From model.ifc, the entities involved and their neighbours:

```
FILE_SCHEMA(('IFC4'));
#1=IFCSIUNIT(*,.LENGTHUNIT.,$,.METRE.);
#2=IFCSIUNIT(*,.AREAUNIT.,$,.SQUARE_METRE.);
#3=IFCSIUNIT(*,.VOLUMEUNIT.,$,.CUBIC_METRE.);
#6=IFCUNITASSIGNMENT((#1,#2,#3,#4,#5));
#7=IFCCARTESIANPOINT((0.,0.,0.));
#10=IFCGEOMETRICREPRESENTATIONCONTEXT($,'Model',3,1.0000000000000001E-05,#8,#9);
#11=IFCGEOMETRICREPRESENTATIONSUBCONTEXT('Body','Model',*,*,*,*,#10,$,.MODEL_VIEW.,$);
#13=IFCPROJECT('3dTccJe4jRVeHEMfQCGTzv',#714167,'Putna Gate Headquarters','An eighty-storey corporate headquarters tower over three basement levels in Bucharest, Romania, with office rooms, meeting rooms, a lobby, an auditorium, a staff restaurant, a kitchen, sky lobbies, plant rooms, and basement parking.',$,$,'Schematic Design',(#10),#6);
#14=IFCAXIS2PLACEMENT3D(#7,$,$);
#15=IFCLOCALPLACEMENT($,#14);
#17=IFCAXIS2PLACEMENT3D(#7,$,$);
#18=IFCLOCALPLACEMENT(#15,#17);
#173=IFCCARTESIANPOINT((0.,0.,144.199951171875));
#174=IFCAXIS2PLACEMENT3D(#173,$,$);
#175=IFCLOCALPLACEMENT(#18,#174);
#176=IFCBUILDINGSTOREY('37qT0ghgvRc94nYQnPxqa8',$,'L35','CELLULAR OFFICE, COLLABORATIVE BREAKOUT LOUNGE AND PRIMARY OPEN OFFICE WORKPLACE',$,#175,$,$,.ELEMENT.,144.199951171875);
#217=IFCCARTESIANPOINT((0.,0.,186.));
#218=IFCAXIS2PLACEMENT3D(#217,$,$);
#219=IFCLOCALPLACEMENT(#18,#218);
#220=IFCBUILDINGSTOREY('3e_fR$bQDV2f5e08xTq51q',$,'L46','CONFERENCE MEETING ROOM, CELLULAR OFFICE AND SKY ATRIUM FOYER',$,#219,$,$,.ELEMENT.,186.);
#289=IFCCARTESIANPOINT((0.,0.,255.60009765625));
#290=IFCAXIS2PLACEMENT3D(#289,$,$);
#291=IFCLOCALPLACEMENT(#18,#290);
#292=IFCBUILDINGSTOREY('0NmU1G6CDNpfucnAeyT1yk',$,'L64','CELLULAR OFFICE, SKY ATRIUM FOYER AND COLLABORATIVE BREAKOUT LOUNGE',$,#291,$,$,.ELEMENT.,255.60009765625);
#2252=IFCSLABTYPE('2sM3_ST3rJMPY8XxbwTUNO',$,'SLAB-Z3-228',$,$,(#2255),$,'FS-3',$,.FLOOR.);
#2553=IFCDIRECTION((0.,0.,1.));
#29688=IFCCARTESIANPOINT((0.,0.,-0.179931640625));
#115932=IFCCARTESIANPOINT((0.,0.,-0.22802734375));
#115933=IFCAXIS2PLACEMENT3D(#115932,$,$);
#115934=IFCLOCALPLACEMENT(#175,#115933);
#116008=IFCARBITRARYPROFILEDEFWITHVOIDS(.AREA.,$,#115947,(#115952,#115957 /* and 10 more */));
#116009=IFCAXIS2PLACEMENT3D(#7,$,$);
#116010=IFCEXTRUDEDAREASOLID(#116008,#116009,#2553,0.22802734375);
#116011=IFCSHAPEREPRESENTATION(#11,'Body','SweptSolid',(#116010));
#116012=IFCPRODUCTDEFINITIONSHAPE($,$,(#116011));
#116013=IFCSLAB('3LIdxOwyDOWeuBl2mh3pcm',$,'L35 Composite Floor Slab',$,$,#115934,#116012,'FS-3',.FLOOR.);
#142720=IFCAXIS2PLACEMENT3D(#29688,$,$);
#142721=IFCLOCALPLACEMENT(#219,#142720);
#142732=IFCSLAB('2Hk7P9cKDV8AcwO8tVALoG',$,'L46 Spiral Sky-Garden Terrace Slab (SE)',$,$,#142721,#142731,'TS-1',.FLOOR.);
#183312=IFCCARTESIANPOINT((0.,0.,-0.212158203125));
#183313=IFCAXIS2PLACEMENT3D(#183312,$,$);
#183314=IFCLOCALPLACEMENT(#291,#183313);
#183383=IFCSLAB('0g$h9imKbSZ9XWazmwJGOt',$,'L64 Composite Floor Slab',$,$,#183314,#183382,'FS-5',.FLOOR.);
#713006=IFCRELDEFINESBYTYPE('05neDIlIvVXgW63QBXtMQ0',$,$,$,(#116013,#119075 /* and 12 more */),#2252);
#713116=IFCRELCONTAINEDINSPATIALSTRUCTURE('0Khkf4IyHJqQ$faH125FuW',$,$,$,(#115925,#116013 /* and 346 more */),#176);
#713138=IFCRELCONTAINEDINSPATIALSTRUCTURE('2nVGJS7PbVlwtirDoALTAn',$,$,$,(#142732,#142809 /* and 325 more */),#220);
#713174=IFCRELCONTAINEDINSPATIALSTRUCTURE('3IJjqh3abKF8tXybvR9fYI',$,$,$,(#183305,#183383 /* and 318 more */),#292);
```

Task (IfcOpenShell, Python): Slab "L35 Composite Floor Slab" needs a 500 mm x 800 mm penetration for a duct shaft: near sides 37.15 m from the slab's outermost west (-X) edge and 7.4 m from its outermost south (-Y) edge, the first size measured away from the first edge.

```python
import numpy as np
import ifcopenshell
import ifcopenshell.api.feature
import ifcopenshell.api.geometry
import ifcopenshell.api.root
import ifcopenshell.geom
import ifcopenshell.util.placement
import ifcopenshell.util.representation
import ifcopenshell.util.shape
import ifcopenshell.util.unit

model = ifcopenshell.open("model.ifc")
unit_scale = ifcopenshell.util.unit.calculate_unit_scale(model)
settings = ifcopenshell.geom.settings()


def volume(element):
    """Net volume in cubic metres, openings subtracted."""
    shape = ifcopenshell.geom.create_shape(settings, element)
    return ifcopenshell.util.shape.get_volume(shape.geometry)


slab = model.by_guid("3LIdxOwyDOWeuBl2mh3pcm")
before = volume(slab)

# Extent in the slab's own axes, in metres. The edges named are its -X and -Y sides.
slab_shape = ifcopenshell.geom.create_shape(settings, slab)
vertices = ifcopenshell.util.shape.get_vertices(slab_shape.geometry)
x_min, y_min, bottom = vertices.min(axis=0)
top = vertices[:, 2].max()

opening = ifcopenshell.api.root.create_entity(model, ifc_class="IfcOpeningElement", name="Duct shaft opening", predefined_type="OPENING")
context = ifcopenshell.util.representation.get_context(model, "Model", "Body", "MODEL_VIEW")
width, depth = 0.5, 0.8
outline = [(0.0, 0.0), (width, 0.0), (width, depth), (0.0, depth), (0.0, 0.0)]
# Overshoot both faces by 50 mm so the cut is clean.
shape = ifcopenshell.api.geometry.add_slab_representation(
    model, context=context, depth=top - bottom + 0.1, polyline=outline
)
ifcopenshell.api.geometry.assign_representation(model, product=opening, representation=shape)

matrix = ifcopenshell.util.placement.get_local_placement(slab.ObjectPlacement)
matrix[:, 3] = matrix @ np.append(np.array([x_min + 37.15, y_min + 7.4, bottom - 0.05]) / unit_scale, 1.0)
ifcopenshell.api.geometry.edit_object_placement(model, product=opening, matrix=matrix, is_si=False)
ifcopenshell.api.feature.add_feature(model, feature=opening, element=slab)

after = volume(slab)

print(f"slab volume {before:.3f} -> {after:.3f} m3")

model.write("model_v2.ifc")
```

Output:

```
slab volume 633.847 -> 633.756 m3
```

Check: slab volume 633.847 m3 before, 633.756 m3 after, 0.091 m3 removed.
